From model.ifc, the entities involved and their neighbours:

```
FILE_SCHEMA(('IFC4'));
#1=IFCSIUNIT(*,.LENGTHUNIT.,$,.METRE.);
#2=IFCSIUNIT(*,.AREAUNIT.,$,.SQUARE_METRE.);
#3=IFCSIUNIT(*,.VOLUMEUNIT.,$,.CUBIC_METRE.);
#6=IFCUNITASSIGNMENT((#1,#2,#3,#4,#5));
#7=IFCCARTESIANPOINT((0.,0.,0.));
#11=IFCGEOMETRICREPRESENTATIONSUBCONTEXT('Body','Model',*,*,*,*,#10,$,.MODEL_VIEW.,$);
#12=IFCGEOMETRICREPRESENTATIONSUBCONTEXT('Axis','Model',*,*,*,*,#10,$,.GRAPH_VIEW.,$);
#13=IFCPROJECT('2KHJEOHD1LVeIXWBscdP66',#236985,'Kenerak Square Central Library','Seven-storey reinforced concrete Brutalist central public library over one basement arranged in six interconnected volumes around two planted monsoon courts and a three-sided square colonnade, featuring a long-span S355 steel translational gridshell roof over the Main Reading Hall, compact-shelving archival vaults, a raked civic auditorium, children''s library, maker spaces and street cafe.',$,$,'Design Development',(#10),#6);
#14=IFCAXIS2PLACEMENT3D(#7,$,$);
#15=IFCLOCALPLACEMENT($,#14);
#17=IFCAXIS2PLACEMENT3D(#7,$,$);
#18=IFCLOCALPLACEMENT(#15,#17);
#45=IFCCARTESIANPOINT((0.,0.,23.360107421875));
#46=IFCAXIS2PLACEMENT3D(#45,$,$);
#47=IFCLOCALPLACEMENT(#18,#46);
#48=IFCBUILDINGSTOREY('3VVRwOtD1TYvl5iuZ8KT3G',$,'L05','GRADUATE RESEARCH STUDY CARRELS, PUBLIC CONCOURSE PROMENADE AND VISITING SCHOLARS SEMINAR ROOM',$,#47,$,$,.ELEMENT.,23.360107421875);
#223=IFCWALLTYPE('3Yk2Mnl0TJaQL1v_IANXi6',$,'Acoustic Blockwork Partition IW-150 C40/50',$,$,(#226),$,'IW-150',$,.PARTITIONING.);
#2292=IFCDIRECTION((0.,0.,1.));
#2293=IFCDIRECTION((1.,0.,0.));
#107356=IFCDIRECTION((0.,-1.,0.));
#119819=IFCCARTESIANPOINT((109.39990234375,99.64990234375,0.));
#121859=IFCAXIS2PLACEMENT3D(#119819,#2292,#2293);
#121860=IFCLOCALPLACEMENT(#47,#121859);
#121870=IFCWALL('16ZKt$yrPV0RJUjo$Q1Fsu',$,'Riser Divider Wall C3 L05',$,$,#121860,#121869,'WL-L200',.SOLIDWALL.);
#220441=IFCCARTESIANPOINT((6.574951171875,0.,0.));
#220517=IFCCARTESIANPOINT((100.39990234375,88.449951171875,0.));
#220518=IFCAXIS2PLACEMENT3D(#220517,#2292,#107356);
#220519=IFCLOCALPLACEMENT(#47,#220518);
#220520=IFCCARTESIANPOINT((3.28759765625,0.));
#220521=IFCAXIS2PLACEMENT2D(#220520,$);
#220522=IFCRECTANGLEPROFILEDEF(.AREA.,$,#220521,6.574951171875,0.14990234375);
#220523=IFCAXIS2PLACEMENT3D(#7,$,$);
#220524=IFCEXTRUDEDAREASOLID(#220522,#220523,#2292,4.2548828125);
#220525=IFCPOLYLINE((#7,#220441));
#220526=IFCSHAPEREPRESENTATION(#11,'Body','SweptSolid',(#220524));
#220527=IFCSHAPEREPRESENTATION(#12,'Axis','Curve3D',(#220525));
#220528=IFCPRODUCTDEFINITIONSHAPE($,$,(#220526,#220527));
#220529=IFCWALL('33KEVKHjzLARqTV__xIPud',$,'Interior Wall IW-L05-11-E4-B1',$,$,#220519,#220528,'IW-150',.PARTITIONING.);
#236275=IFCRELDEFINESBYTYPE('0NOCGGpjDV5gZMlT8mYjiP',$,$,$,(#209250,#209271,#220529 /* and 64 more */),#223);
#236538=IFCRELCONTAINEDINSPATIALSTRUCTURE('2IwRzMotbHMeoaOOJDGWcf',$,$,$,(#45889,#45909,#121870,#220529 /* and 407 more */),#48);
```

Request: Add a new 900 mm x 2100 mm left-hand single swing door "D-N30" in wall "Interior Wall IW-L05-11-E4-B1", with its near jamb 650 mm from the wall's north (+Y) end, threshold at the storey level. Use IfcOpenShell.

```python
import numpy as np
import ifcopenshell
import ifcopenshell.api.feature
import ifcopenshell.api.geometry
import ifcopenshell.api.root
import ifcopenshell.api.spatial
import ifcopenshell.geom
import ifcopenshell.util.element
import ifcopenshell.util.placement
import ifcopenshell.util.representation
import ifcopenshell.util.shape
import ifcopenshell.util.unit

model = ifcopenshell.open("model.ifc")
unit_scale = ifcopenshell.util.unit.calculate_unit_scale(model)
settings = ifcopenshell.geom.settings()


def volume(element):
    """Net volume in cubic metres, openings subtracted."""
    shape = ifcopenshell.geom.create_shape(settings, element)
    return ifcopenshell.util.shape.get_volume(shape.geometry)


wall = model.by_id(220529)
storey = ifcopenshell.util.element.get_container(wall, ifc_class="IfcBuildingStorey")
context = ifcopenshell.util.representation.get_context(model, "Model", "Body", "MODEL_VIEW")
before = volume(wall)

width, height, from_end, sill = 0.9, 2.1, 0.65, 0.0  # metres

# The wall runs along its own X axis, and the end named is its -X end.
wall_shape = ifcopenshell.geom.create_shape(settings, wall)
x, y, z = ifcopenshell.util.shape.get_vertices(wall_shape.geometry).T
start = x.min() + from_end
face, thickness = float(y.min()), float(y.max() - y.min())
wall_matrix = ifcopenshell.util.placement.get_local_placement(wall.ObjectPlacement)
level = ifcopenshell.util.placement.get_local_placement(storey.ObjectPlacement)[2, 3]


def in_wall(x, y):
    """Placement at x, y metres in the wall's axes, at sill height."""
    matrix = wall_matrix.copy()
    matrix[:, 3] = wall_matrix @ np.array([x / unit_scale, y / unit_scale, 0.0, 1.0])
    matrix[2, 3] = level + sill / unit_scale
    return matrix


# Opening: a box that overshoots both wall faces by 50 mm.
opening = ifcopenshell.api.root.create_entity(model, ifc_class="IfcOpeningElement", predefined_type="OPENING")
box = ifcopenshell.api.geometry.add_wall_representation(
    model, context=context, length=width, height=height, thickness=thickness + 0.1
)
ifcopenshell.api.geometry.assign_representation(model, product=opening, representation=box)
ifcopenshell.api.geometry.edit_object_placement(model, product=opening, matrix=in_wall(start, face - 0.05), is_si=False)
ifcopenshell.api.feature.add_feature(model, feature=opening, element=wall)

door = ifcopenshell.api.root.create_entity(model, ifc_class="IfcDoor", name="D-N30", predefined_type="DOOR")
door.OverallWidth, door.OverallHeight = width / unit_scale, height / unit_scale
door.OperationType = "SINGLE_SWING_LEFT"
body = ifcopenshell.api.geometry.add_door_representation(
    model,
    context=context,
    overall_width=door.OverallWidth,
    overall_height=door.OverallHeight,
    operation_type="SINGLE_SWING_LEFT",
    lining_properties={"LiningDepth": thickness / unit_scale, "ThresholdDepth": thickness / unit_scale},
)
ifcopenshell.api.geometry.assign_representation(model, product=door, representation=body)
ifcopenshell.api.spatial.assign_container(model, products=[door], relating_structure=storey)
ifcopenshell.api.feature.add_filling(model, opening=opening, element=door)

# The lining spans the wall, so the door starts at the wall face.
ifcopenshell.api.geometry.edit_object_placement(model, product=door, matrix=in_wall(start, face), is_si=False)

after = volume(wall)

print(f"wall volume {before:.3f} -> {after:.3f} m3")

model.write("model_edited.ifc")
```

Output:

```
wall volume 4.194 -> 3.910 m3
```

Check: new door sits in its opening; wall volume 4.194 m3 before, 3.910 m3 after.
